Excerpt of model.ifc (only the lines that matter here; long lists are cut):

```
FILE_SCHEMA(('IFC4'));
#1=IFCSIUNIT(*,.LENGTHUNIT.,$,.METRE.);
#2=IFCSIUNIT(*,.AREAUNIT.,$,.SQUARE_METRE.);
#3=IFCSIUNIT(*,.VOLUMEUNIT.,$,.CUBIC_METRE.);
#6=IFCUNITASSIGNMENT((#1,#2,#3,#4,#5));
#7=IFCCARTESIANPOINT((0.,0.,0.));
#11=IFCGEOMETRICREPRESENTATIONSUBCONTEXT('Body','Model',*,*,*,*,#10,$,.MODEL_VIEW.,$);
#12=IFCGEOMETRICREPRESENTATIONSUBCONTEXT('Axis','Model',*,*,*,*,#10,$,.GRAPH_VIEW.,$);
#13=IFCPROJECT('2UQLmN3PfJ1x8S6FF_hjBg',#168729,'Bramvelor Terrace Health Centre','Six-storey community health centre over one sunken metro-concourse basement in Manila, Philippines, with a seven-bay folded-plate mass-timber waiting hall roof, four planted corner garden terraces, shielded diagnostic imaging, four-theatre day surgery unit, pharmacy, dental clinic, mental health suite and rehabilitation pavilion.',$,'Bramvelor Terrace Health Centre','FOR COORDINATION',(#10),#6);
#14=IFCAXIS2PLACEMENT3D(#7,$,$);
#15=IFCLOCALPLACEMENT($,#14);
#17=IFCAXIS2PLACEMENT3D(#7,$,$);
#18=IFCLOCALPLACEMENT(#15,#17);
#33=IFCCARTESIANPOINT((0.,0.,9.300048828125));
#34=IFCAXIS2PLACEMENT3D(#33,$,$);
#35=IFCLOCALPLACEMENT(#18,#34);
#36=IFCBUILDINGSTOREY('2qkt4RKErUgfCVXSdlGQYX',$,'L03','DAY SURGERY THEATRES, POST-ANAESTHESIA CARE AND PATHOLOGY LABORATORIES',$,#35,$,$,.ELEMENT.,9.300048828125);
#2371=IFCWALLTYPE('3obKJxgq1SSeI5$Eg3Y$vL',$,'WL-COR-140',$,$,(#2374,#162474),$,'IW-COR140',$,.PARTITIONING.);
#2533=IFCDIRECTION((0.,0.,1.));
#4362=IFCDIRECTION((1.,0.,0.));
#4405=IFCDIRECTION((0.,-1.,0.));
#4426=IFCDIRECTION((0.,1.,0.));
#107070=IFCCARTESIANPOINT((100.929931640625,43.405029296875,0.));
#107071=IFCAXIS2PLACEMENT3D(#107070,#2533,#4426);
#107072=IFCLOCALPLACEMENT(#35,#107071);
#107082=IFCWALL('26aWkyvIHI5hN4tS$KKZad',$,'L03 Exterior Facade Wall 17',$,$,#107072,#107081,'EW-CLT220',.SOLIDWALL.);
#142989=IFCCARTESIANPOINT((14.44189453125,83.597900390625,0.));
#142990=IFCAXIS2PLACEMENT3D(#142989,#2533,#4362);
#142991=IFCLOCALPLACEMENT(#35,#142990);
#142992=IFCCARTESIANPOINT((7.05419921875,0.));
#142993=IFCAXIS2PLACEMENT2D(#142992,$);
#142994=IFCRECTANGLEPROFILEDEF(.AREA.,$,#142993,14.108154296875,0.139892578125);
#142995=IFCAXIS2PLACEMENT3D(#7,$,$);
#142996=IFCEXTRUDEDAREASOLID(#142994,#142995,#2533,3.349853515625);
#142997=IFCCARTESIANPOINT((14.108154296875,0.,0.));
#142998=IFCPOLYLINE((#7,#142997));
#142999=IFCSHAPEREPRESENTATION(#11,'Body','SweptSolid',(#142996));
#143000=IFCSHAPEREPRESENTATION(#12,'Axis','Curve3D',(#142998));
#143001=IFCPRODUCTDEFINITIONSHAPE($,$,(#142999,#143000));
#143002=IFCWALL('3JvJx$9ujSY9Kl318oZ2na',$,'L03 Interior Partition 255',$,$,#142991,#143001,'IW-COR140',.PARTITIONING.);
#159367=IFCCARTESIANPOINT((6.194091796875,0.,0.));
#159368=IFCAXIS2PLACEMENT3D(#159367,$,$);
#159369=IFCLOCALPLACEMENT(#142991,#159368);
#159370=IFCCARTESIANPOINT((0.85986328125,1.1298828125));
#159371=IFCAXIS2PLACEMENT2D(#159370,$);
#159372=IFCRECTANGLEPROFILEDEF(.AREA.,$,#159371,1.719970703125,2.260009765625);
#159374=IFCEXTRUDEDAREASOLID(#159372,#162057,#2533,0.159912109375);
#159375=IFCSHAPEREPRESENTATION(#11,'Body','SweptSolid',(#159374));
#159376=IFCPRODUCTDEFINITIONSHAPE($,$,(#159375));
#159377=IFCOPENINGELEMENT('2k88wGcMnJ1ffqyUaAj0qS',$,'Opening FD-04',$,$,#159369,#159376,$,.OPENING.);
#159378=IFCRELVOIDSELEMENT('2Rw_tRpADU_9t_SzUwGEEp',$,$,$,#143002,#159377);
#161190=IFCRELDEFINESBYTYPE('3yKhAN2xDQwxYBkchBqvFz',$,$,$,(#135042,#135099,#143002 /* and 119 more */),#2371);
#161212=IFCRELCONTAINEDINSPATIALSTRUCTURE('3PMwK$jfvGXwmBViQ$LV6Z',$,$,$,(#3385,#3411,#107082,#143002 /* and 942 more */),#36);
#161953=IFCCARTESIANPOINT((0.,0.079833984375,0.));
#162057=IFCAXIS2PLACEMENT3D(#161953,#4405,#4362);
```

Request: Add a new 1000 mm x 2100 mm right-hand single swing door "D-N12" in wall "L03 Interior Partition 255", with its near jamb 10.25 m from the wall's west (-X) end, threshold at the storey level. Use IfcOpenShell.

```python
import numpy as np
import ifcopenshell
import ifcopenshell.api.feature
import ifcopenshell.api.geometry
import ifcopenshell.api.root
import ifcopenshell.api.spatial
import ifcopenshell.geom
import ifcopenshell.util.element
import ifcopenshell.util.placement
import ifcopenshell.util.representation
import ifcopenshell.util.shape
import ifcopenshell.util.unit

model = ifcopenshell.open("model.ifc")
unit_scale = ifcopenshell.util.unit.calculate_unit_scale(model)
settings = ifcopenshell.geom.settings()


def volume(element):
    """Net volume in cubic metres, openings subtracted."""
    shape = ifcopenshell.geom.create_shape(settings, element)
    return ifcopenshell.util.shape.get_volume(shape.geometry)


wall = model.by_guid("3JvJx$9ujSY9Kl318oZ2na")
storey = ifcopenshell.util.element.get_container(wall, ifc_class="IfcBuildingStorey")
context = ifcopenshell.util.representation.get_context(model, "Model", "Body", "MODEL_VIEW")
before = volume(wall)

width, height, from_end, sill = 1, 2.1, 10.25, 0.0  # metres

# The wall runs along its own X axis, and the end named is its -X end.
wall_shape = ifcopenshell.geom.create_shape(settings, wall)
x, y, z = ifcopenshell.util.shape.get_vertices(wall_shape.geometry).T
start = x.min() + from_end
face, thickness = float(y.min()), float(y.max() - y.min())
wall_matrix = ifcopenshell.util.placement.get_local_placement(wall.ObjectPlacement)
level = ifcopenshell.util.placement.get_local_placement(storey.ObjectPlacement)[2, 3]


def in_wall(x, y):
    """Placement at x, y metres in the wall's axes, at sill height."""
    matrix = wall_matrix.copy()
    matrix[:, 3] = wall_matrix @ np.array([x / unit_scale, y / unit_scale, 0.0, 1.0])
    matrix[2, 3] = level + sill / unit_scale
    return matrix


# Opening: a box that overshoots both wall faces by 50 mm.
opening = ifcopenshell.api.root.create_entity(model, ifc_class="IfcOpeningElement", predefined_type="OPENING")
box = ifcopenshell.api.geometry.add_wall_representation(
    model, context=context, length=width, height=height, thickness=thickness + 0.1
)
ifcopenshell.api.geometry.assign_representation(model, product=opening, representation=box)
ifcopenshell.api.geometry.edit_object_placement(model, product=opening, matrix=in_wall(start, face - 0.05), is_si=False)
ifcopenshell.api.feature.add_feature(model, feature=opening, element=wall)

door = ifcopenshell.api.root.create_entity(model, ifc_class="IfcDoor", name="D-N12", predefined_type="DOOR")
door.OverallWidth, door.OverallHeight = width / unit_scale, height / unit_scale
door.OperationType = "SINGLE_SWING_RIGHT"
body = ifcopenshell.api.geometry.add_door_representation(
    model,
    context=context,
    overall_width=door.OverallWidth,
    overall_height=door.OverallHeight,
    operation_type="SINGLE_SWING_RIGHT",
    lining_properties={"LiningDepth": thickness / unit_scale, "ThresholdDepth": thickness / unit_scale},
)
ifcopenshell.api.geometry.assign_representation(model, product=door, representation=body)
ifcopenshell.api.spatial.assign_container(model, products=[door], relating_structure=storey)
ifcopenshell.api.feature.add_filling(model, opening=opening, element=door)

# The lining spans the wall, so the door starts at the wall face.
ifcopenshell.api.geometry.edit_object_placement(model, product=door, matrix=in_wall(start, face), is_si=False)

after = volume(wall)

print(f"wall volume {before:.3f} -> {after:.3f} m3")

model.write("model-out.ifc")
```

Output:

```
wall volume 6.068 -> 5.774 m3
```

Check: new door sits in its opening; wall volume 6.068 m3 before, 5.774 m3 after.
